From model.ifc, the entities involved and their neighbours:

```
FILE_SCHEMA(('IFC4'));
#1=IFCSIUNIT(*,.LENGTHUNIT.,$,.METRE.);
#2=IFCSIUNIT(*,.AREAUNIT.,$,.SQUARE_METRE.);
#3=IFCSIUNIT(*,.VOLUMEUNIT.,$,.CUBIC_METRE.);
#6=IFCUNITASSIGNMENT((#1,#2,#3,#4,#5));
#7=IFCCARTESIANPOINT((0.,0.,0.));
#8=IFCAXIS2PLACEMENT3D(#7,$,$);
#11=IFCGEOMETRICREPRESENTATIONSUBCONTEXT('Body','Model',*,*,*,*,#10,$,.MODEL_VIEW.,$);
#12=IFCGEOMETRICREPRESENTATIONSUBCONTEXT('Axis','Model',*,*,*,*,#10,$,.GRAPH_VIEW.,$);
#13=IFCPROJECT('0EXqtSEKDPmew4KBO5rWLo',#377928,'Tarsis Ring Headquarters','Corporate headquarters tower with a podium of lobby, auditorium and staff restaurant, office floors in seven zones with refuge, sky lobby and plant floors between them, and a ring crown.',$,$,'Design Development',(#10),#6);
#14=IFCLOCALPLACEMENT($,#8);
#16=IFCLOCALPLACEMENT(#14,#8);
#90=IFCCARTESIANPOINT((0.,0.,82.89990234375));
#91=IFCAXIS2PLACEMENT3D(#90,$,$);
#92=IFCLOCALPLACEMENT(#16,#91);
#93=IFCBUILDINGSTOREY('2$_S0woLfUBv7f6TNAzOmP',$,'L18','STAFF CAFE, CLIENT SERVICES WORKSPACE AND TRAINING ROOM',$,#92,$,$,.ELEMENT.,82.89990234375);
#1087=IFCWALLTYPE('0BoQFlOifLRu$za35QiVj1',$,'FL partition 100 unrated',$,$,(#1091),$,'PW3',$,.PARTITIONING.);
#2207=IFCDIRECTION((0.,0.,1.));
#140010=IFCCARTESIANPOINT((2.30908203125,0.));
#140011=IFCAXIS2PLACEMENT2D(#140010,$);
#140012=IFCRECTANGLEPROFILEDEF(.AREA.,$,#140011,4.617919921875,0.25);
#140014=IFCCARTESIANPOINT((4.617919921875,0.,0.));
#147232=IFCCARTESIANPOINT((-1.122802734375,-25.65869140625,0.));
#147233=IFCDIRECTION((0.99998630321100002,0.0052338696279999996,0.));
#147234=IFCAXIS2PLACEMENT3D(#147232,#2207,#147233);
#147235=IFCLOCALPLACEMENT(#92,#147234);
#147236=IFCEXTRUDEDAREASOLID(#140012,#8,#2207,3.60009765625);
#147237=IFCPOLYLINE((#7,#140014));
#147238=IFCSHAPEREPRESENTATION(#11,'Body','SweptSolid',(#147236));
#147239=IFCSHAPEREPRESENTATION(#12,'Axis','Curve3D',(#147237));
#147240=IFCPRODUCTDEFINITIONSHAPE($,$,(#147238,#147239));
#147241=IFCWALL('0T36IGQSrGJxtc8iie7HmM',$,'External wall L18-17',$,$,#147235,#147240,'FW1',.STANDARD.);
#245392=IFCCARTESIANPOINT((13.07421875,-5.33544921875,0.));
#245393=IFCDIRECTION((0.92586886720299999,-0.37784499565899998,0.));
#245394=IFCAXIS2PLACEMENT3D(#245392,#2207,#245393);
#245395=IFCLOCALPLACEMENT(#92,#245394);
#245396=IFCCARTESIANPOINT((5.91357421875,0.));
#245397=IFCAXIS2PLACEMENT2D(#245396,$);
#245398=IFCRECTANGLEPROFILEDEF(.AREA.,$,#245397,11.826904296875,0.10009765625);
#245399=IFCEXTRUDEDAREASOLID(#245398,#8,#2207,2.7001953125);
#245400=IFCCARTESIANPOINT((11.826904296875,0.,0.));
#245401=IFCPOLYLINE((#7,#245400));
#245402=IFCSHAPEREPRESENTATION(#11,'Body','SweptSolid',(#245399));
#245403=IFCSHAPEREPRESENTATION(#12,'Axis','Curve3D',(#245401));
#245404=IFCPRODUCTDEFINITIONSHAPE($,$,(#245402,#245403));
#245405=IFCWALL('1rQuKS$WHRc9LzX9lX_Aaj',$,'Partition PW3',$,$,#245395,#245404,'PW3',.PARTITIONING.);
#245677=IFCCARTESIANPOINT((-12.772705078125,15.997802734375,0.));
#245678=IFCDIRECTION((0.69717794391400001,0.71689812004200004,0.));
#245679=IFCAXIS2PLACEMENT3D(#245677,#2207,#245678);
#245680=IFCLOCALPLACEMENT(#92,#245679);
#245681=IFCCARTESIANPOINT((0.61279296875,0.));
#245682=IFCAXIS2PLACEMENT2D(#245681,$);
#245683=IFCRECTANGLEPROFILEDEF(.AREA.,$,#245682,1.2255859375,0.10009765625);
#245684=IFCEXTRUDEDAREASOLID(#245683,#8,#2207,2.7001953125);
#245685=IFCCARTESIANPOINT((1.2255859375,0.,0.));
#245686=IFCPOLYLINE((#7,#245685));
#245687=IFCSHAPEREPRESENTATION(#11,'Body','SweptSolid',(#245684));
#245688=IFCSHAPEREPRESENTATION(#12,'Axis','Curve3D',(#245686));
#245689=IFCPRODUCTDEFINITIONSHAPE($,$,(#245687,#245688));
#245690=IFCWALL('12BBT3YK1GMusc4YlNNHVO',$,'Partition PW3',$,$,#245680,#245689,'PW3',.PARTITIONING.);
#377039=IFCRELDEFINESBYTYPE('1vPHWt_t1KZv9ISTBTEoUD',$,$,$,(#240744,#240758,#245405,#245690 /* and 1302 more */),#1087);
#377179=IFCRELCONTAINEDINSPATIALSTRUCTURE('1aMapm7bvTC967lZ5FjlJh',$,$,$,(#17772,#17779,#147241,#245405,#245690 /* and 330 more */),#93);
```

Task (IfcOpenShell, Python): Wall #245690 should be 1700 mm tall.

```python
import ifcopenshell
import ifcopenshell.geom
import ifcopenshell.util.representation
import ifcopenshell.util.shape

model = ifcopenshell.open("model.ifc")
settings = ifcopenshell.geom.settings()


def volume(element):
    """Net volume in cubic metres, openings subtracted."""
    shape = ifcopenshell.geom.create_shape(settings, element)
    return ifcopenshell.util.shape.get_volume(shape.geometry)


wall = model.by_id(245690)
before = volume(wall)

body = ifcopenshell.util.representation.get_representation(wall, "Model", "Body")
solid = body.Items[0]
old_height = solid.Depth
solid.Depth = 1.7
after = volume(wall)

print(f"height {old_height:g} -> {solid.Depth:g}, volume {before:.3f} -> {after:.3f} m3")

model.write("model-out.ifc")
```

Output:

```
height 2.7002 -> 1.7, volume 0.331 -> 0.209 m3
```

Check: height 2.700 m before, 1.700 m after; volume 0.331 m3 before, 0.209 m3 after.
